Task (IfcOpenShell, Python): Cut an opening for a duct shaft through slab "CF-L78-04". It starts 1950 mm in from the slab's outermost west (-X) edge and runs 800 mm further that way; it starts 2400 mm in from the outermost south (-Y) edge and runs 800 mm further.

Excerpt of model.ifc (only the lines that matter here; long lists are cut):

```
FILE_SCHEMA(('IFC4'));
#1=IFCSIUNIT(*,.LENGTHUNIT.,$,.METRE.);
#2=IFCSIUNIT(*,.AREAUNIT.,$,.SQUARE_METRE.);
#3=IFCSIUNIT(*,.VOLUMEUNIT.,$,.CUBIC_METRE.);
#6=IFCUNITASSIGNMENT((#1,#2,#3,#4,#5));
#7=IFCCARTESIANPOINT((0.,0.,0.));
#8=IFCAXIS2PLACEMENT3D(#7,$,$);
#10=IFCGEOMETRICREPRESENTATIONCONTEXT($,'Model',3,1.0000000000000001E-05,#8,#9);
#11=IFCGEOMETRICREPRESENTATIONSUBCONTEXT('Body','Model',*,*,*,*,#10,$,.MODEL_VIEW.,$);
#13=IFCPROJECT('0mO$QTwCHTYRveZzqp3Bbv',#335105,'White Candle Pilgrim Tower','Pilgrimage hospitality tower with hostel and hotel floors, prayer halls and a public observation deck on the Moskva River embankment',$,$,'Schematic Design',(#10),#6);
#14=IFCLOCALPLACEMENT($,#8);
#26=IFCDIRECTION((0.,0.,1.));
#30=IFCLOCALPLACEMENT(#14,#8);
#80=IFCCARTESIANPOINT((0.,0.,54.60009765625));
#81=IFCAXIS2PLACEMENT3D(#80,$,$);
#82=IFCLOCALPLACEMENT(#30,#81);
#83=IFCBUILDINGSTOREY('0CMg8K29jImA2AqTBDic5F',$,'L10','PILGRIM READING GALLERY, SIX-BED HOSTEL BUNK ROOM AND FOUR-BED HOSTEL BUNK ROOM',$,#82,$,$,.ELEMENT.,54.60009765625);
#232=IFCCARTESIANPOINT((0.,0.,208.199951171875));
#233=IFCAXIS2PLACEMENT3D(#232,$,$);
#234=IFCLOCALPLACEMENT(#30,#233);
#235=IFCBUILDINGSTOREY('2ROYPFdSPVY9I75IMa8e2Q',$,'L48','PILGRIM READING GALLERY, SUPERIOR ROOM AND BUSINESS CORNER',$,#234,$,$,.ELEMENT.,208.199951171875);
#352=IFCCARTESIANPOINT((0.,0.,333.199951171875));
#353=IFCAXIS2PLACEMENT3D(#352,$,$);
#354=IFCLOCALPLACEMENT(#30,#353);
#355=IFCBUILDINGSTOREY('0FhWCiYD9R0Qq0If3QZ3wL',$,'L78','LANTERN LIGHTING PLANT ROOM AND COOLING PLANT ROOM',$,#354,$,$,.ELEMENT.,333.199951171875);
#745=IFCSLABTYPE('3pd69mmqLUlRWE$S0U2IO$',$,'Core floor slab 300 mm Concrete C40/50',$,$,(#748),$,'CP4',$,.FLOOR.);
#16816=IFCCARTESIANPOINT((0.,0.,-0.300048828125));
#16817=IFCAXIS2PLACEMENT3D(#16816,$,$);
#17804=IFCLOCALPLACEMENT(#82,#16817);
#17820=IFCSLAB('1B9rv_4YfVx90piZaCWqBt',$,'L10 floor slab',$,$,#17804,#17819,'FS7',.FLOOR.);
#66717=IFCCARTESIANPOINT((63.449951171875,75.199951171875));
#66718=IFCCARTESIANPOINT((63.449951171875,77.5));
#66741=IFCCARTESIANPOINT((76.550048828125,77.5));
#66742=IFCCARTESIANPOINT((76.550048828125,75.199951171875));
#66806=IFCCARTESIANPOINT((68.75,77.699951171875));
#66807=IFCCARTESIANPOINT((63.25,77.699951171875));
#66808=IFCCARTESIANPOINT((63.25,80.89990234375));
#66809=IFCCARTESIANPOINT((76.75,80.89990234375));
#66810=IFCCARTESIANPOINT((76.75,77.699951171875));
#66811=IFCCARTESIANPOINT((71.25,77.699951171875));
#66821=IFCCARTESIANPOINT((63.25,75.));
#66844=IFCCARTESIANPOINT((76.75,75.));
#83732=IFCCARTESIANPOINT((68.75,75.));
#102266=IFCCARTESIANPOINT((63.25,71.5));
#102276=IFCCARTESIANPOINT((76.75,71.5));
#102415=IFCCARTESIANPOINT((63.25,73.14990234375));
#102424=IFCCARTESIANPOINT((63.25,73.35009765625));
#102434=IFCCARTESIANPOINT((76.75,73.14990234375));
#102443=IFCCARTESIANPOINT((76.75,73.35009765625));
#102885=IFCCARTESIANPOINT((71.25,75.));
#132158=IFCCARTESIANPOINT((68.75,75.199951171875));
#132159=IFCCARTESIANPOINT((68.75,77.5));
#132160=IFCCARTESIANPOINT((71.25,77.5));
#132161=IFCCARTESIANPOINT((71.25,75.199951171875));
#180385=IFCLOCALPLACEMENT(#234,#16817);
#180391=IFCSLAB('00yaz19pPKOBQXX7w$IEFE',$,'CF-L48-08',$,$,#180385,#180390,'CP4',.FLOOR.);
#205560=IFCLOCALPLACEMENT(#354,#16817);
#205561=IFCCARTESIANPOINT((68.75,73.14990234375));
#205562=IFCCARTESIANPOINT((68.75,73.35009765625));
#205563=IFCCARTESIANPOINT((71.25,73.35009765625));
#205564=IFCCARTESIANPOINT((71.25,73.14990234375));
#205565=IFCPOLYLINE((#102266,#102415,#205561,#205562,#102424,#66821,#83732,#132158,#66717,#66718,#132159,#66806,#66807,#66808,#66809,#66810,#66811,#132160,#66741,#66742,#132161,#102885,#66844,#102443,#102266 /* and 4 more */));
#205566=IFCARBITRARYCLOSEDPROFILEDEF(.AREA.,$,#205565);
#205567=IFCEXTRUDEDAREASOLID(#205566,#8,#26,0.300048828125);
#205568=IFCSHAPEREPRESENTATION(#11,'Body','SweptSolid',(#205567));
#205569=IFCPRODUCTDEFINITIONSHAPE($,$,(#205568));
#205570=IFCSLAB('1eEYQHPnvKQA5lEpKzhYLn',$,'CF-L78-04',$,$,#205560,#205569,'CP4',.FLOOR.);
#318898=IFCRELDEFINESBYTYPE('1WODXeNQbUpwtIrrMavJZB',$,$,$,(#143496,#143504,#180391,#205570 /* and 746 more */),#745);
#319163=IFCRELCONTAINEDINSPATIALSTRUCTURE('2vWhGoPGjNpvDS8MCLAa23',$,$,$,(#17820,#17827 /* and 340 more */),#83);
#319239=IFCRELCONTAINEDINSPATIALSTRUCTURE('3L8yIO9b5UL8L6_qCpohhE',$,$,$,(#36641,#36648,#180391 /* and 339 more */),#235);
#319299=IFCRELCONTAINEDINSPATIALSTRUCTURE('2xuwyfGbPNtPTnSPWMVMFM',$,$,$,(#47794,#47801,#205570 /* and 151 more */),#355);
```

```python
import numpy as np
import ifcopenshell
import ifcopenshell.api.feature
import ifcopenshell.api.geometry
import ifcopenshell.api.root
import ifcopenshell.geom
import ifcopenshell.util.placement
import ifcopenshell.util.representation
import ifcopenshell.util.shape
import ifcopenshell.util.unit

model = ifcopenshell.open("model.ifc")
unit_scale = ifcopenshell.util.unit.calculate_unit_scale(model)
settings = ifcopenshell.geom.settings()


def volume(element):
    """Net volume in cubic metres, openings subtracted."""
    shape = ifcopenshell.geom.create_shape(settings, element)
    return ifcopenshell.util.shape.get_volume(shape.geometry)


slab = model.by_guid("1eEYQHPnvKQA5lEpKzhYLn")
before = volume(slab)

# Extent in the slab's own axes, in metres. The edges named are its -X and -Y sides.
slab_shape = ifcopenshell.geom.create_shape(settings, slab)
vertices = ifcopenshell.util.shape.get_vertices(slab_shape.geometry)
x_min, y_min, bottom = vertices.min(axis=0)
top = vertices[:, 2].max()

opening = ifcopenshell.api.root.create_entity(model, ifc_class="IfcOpeningElement", name="Duct shaft opening", predefined_type="OPENING")
context = ifcopenshell.util.representation.get_context(model, "Model", "Body", "MODEL_VIEW")
width, depth = 0.8, 0.8
outline = [(0.0, 0.0), (width, 0.0), (width, depth), (0.0, depth), (0.0, 0.0)]
# Overshoot both faces by 50 mm so the cut is clean.
shape = ifcopenshell.api.geometry.add_slab_representation(
    model, context=context, depth=top - bottom + 0.1, polyline=outline
)
ifcopenshell.api.geometry.assign_representation(model, product=opening, representation=shape)

matrix = ifcopenshell.util.placement.get_local_placement(slab.ObjectPlacement)
matrix[:, 3] = matrix @ np.append(np.array([x_min + 1.95, y_min + 2.4, bottom - 0.05]) / unit_scale, 1.0)
ifcopenshell.api.geometry.edit_object_placement(model, product=opening, matrix=matrix, is_si=False)
ifcopenshell.api.feature.add_feature(model, feature=opening, element=slab)

after = volume(slab)

print(f"slab volume {before:.3f} -> {after:.3f} m3")

model.write("model_v2.ifc")
```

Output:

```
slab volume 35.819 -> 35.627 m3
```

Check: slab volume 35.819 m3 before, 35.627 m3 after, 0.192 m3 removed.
